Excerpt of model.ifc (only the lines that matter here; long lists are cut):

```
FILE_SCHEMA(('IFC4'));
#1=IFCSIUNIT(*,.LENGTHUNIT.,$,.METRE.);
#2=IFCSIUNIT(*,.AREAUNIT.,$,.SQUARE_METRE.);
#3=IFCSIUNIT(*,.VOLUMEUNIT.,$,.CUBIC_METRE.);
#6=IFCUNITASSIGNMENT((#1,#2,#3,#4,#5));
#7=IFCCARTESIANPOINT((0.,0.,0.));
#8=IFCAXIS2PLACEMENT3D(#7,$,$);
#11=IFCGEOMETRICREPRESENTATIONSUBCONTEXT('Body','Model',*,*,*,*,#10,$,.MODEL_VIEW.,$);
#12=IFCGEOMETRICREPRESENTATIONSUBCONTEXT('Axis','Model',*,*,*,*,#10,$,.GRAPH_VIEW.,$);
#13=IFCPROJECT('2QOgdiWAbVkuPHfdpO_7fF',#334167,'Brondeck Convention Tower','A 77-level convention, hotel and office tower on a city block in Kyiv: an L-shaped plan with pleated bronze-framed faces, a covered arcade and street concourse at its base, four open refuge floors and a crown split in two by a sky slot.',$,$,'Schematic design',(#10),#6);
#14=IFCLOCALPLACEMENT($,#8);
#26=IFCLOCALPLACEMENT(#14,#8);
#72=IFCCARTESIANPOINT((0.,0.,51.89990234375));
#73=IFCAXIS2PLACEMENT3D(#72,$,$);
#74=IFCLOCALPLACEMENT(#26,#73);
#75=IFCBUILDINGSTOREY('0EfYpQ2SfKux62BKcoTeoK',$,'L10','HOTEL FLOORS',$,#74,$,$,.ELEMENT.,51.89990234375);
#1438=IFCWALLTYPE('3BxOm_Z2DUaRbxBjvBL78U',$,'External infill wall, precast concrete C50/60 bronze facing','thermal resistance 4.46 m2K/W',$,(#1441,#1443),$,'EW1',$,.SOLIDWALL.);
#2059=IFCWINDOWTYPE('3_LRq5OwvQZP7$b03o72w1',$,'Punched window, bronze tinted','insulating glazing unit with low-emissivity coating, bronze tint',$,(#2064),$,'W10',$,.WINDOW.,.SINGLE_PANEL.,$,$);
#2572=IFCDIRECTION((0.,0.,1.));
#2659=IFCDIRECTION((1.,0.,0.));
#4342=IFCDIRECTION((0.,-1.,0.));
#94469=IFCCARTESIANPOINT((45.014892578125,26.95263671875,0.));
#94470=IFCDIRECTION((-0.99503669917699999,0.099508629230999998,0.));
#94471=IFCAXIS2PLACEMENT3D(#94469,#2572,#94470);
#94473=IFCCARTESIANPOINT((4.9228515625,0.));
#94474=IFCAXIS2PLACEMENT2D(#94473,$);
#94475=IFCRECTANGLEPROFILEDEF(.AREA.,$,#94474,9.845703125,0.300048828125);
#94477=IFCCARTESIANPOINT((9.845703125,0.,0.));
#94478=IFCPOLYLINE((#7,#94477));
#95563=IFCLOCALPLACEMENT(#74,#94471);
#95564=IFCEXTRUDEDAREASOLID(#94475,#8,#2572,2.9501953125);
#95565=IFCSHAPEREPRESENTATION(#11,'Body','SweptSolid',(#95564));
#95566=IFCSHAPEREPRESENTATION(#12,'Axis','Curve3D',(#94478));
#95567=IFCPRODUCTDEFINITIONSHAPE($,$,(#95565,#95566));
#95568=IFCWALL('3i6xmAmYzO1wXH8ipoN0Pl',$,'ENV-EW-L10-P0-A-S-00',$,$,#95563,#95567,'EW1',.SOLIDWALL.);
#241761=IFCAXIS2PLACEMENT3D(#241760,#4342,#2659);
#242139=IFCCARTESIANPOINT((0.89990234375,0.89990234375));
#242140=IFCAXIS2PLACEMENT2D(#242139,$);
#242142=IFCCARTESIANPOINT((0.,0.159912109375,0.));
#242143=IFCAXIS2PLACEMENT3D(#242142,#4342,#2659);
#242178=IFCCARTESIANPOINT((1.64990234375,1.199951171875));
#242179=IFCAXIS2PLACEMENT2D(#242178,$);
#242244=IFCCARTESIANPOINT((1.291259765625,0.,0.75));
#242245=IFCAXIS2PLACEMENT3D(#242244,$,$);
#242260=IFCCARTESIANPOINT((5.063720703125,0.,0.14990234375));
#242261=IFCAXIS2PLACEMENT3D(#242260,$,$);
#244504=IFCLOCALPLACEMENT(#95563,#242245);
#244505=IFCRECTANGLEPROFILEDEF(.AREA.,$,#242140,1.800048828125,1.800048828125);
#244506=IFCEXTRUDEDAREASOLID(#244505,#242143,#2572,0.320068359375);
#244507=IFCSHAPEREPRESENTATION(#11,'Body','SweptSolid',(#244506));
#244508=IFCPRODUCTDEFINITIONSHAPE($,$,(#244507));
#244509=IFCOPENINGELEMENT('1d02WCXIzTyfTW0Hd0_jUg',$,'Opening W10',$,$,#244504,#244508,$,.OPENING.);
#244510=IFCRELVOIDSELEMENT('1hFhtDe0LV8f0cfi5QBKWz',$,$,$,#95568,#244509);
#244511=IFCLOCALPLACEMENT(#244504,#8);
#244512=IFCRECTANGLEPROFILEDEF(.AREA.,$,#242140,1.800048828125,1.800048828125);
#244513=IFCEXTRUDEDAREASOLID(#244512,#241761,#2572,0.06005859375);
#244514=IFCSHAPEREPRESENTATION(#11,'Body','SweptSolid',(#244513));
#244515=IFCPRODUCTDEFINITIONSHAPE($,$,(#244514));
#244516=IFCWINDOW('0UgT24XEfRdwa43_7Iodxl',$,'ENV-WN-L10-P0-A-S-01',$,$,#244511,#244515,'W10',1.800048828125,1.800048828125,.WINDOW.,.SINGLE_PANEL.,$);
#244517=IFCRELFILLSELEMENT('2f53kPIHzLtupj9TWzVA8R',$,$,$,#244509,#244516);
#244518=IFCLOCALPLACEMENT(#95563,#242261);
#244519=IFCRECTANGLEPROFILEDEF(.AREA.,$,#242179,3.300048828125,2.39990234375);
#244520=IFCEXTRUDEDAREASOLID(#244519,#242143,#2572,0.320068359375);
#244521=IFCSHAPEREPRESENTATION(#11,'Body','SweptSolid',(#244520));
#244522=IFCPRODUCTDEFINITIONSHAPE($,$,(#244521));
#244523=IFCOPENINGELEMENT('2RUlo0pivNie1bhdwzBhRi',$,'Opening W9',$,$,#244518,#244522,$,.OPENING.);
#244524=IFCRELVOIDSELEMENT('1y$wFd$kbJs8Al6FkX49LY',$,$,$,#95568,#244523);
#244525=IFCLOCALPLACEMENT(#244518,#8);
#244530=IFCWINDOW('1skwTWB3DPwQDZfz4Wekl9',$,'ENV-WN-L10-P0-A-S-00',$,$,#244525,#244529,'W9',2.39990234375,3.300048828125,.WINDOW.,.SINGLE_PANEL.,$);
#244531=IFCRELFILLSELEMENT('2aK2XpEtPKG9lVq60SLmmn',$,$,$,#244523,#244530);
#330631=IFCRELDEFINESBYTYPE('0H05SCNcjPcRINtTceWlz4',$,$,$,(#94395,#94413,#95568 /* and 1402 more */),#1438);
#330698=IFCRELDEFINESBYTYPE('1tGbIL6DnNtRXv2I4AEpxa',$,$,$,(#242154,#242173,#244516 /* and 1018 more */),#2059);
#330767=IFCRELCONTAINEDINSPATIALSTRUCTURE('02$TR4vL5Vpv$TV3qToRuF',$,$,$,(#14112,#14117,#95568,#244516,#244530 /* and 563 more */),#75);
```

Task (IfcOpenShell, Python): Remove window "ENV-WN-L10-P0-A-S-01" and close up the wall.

```python
import ifcopenshell
import ifcopenshell.api.feature
import ifcopenshell.api.root
import ifcopenshell.geom
import ifcopenshell.util.shape

model = ifcopenshell.open("model.ifc")
settings = ifcopenshell.geom.settings()


def volume(element):
    """Net volume in cubic metres, openings subtracted."""
    shape = ifcopenshell.geom.create_shape(settings, element)
    return ifcopenshell.util.shape.get_volume(shape.geometry)


window = model.by_guid("0UgT24XEfRdwa43_7Iodxl")
opening = window.FillsVoids[0].RelatingOpeningElement
wall = opening.VoidsElements[0].RelatingBuildingElement
before = volume(wall)

ifcopenshell.api.root.remove_product(model, product=window)
ifcopenshell.api.feature.remove_feature(model, feature=opening)

after = volume(wall)

print(f"wall volume {before:.3f} -> {after:.3f} m3")

model.write("model_rev.ifc")
```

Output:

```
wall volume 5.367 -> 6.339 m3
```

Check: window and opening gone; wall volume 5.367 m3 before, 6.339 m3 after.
